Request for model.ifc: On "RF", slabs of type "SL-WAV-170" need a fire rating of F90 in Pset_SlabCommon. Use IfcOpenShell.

First a look at what the model holds.

```python
import ifcopenshell
import ifcopenshell.util.element

model = ifcopenshell.open("model.ifc")
print(model.schema)
storey = next(s for s in model.by_type("IfcBuildingStorey") if s.Name == "RF")
slabs = [e for e in ifcopenshell.util.element.get_decomposition(storey) if e.is_a("IfcSlab")]
seen = {}
for e in slabs:
    element_type = ifcopenshell.util.element.get_type(e)
    key = (element_type.Name if element_type != e and element_type else None, ifcopenshell.util.element.get_pset(e, "Pset_SlabCommon", "FireRating"))
    seen[key] = seen.get(key, 0) + 1
for (name, value), count in sorted(seen.items(), key=str):
    print(count, "x", name, "|", value)
```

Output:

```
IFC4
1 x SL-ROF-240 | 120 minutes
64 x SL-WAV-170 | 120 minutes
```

```python
import ifcopenshell
import ifcopenshell.api.pset
import ifcopenshell.util.element

model = ifcopenshell.open("model.ifc")

storey = next(s for s in model.by_type("IfcBuildingStorey") if s.Name == "RF")
slabs = [e for e in ifcopenshell.util.element.get_decomposition(storey) if e.is_a("IfcSlab")]

count = 0
for e in slabs:
    element_type = ifcopenshell.util.element.get_type(e)
    if element_type in (None, e) or element_type.Name != "SL-WAV-170":
        continue
    # add_pset returns the element's existing set when there is one.
    pset = ifcopenshell.api.pset.add_pset(model, product=e, name="Pset_SlabCommon")
    ifcopenshell.api.pset.edit_pset(model, pset=pset, properties={"FireRating": "F90"})
    count += 1

print(count, "slabs updated")

model.write("model-out.ifc")
```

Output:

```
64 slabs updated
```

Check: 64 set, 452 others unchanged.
